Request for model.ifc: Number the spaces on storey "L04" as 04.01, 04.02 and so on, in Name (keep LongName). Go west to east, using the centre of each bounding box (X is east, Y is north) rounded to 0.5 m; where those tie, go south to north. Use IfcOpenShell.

First a look at what the model holds.

```python
import ifcopenshell
import ifcopenshell.util.element
import ifcopenshell.util.placement

model = ifcopenshell.open("model.ifc")
print(model.schema)
storey = next(s for s in model.by_type("IfcBuildingStorey") if s.Name == "L04")
spaces = [e for e in ifcopenshell.util.element.get_decomposition(storey) if e.is_a("IfcSpace")]
for e in sorted(spaces, key=lambda e: e.id()):
    origin = ifcopenshell.util.placement.get_local_placement(e.ObjectPlacement)[:3, 3]
    print(e.id(), e.Name, e.LongName, origin.round(2) + 0.0, sep=" | ")
```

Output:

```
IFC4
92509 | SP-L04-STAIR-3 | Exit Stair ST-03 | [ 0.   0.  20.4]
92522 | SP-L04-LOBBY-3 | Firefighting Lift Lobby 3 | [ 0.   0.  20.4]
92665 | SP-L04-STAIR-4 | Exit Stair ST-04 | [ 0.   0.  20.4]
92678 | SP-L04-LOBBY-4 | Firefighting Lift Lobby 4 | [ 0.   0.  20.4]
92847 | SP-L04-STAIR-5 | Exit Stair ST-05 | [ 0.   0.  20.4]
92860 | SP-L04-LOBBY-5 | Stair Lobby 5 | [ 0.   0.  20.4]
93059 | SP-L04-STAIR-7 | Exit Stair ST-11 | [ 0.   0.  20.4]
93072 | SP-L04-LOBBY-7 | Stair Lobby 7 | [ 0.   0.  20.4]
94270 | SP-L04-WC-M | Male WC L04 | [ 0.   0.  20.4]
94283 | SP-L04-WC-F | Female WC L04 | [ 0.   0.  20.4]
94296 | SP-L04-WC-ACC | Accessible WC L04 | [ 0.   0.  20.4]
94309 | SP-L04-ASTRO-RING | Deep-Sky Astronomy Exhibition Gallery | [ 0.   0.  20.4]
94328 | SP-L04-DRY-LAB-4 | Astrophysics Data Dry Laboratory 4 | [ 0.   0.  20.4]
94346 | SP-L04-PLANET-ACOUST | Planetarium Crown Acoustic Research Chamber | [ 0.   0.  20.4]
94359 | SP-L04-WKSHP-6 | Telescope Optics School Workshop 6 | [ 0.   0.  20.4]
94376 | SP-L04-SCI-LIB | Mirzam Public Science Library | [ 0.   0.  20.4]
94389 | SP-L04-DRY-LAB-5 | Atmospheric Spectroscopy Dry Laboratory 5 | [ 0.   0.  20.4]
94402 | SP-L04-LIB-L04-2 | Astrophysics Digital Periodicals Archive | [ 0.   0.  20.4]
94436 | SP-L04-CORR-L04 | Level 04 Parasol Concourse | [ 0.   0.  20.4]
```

```python
import ifcopenshell
import ifcopenshell.geom
import ifcopenshell.util.element
import ifcopenshell.util.shape

model = ifcopenshell.open("model.ifc")
settings = ifcopenshell.geom.settings()
settings.set("use-world-coords", True)


def centre(element):
    shape = ifcopenshell.geom.create_shape(settings, element)
    return ifcopenshell.util.shape.get_bbox_centroid(shape.geometry)


storey = next(s for s in model.by_type("IfcBuildingStorey") if s.Name == "L04")
spaces = [e for e in ifcopenshell.util.element.get_decomposition(storey) if e.is_a("IfcSpace")]

# Insertion points can sit at a corner or the storey origin, so sort by the geometry (in metres).
centres = {e: centre(e) for e in spaces}
spaces.sort(key=lambda e: (round(centres[e][0] / 0.5), centres[e][1]))

for i, e in enumerate(spaces, start=1):
    number = f"04.{i:02d}"
    e.Name = number
    print(e.id(), number)

model.write("model_rev.ifc")
```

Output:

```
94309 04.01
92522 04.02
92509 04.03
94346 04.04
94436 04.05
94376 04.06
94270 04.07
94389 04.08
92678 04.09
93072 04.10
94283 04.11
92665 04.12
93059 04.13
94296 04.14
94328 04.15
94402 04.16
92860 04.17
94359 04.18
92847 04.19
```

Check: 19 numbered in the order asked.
